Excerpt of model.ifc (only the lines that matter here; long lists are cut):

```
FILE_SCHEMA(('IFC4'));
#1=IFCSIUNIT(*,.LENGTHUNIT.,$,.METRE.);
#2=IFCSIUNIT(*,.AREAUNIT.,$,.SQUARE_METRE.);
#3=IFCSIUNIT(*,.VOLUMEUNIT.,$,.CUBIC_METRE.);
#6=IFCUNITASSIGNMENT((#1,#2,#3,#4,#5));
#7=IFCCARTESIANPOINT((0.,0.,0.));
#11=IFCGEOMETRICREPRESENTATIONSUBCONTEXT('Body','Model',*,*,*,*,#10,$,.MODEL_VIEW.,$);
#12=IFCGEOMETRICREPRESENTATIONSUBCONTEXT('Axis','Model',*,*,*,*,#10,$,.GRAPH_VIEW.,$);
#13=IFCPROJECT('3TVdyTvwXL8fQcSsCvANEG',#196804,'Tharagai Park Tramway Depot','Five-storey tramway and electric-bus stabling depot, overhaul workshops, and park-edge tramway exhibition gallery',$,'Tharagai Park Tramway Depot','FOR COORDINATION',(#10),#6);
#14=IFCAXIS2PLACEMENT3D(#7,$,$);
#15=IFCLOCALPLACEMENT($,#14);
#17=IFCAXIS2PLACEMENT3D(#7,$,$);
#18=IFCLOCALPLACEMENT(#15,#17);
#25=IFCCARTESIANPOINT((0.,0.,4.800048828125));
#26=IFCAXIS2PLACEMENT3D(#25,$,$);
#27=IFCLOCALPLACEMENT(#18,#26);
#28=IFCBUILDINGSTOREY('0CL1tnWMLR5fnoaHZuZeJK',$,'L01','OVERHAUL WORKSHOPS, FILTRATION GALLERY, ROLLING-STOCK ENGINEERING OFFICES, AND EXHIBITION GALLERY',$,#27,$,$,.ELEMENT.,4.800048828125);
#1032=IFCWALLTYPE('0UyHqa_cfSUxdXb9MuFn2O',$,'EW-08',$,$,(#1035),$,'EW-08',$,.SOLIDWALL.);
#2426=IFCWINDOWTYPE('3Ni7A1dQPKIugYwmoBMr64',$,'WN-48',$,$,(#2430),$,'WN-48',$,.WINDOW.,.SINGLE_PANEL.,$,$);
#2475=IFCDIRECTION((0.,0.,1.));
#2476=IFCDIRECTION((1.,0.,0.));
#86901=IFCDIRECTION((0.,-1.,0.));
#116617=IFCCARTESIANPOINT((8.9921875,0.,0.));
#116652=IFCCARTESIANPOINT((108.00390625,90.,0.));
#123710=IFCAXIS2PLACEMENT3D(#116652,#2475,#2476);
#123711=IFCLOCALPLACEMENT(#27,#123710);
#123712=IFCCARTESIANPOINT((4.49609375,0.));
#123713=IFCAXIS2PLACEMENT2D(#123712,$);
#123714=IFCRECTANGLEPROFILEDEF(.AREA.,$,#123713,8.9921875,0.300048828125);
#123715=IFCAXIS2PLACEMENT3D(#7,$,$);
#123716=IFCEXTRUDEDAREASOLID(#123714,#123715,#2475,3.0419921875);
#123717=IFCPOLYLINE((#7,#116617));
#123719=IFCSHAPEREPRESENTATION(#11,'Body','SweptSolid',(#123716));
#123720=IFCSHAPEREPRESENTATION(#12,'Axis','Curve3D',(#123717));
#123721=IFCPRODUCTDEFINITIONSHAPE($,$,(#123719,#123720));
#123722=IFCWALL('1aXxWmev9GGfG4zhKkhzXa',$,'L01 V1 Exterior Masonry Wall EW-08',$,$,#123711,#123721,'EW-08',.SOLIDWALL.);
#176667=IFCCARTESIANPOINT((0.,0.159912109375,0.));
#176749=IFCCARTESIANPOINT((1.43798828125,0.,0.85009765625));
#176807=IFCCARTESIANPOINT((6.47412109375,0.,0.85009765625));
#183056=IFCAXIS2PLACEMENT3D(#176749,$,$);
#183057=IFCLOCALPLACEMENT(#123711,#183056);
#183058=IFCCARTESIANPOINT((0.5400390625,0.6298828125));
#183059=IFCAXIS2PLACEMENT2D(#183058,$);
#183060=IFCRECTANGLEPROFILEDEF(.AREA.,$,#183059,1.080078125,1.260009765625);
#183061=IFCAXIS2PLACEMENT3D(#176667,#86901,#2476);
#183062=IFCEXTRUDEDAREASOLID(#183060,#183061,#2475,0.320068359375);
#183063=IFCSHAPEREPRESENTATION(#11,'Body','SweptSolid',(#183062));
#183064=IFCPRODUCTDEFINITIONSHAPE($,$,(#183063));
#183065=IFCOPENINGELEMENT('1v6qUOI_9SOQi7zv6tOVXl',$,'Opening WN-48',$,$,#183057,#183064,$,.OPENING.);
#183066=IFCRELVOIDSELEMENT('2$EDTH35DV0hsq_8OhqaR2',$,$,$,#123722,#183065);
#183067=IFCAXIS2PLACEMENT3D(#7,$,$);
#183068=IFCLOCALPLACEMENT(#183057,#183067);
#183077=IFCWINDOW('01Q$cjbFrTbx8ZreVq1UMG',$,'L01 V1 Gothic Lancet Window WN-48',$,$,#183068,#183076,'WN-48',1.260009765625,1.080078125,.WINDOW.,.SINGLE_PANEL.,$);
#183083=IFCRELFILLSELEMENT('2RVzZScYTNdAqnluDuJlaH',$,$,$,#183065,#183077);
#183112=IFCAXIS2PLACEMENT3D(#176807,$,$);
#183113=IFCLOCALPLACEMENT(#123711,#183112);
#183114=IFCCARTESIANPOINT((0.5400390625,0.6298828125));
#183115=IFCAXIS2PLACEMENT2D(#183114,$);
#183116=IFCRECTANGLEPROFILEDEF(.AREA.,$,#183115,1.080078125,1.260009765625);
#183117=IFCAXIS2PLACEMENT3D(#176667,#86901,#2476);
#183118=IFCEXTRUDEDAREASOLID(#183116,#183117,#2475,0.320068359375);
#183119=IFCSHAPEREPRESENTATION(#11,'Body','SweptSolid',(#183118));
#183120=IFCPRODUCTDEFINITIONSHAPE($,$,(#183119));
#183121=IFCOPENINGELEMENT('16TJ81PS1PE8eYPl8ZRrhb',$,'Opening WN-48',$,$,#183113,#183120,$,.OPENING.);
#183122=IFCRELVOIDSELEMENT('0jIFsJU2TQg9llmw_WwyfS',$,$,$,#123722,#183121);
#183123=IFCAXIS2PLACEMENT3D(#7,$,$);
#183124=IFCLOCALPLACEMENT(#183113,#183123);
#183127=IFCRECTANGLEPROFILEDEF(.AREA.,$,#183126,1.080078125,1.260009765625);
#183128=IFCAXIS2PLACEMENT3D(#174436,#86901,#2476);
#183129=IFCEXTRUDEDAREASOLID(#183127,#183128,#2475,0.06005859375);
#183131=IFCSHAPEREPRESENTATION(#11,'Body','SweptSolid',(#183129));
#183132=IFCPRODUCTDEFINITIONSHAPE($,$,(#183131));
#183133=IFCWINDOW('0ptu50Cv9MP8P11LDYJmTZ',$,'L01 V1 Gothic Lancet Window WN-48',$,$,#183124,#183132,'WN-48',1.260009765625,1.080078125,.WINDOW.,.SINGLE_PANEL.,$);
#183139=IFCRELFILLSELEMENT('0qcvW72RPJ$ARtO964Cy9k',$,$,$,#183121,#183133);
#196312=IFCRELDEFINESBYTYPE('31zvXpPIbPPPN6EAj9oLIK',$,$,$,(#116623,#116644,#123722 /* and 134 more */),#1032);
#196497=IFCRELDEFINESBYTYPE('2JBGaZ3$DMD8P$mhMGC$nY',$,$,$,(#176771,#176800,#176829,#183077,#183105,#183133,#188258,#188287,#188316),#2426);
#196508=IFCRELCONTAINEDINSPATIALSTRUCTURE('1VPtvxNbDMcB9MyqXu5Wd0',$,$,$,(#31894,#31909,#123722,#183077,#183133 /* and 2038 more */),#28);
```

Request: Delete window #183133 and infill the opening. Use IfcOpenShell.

```python
import ifcopenshell
import ifcopenshell.api.feature
import ifcopenshell.api.root
import ifcopenshell.geom
import ifcopenshell.util.shape

model = ifcopenshell.open("model.ifc")
settings = ifcopenshell.geom.settings()


def volume(element):
    """Net volume in cubic metres, openings subtracted."""
    shape = ifcopenshell.geom.create_shape(settings, element)
    return ifcopenshell.util.shape.get_volume(shape.geometry)


window = model.by_guid("0ptu50Cv9MP8P11LDYJmTZ")
opening = window.FillsVoids[0].RelatingOpeningElement
wall = opening.VoidsElements[0].RelatingBuildingElement
before = volume(wall)

ifcopenshell.api.root.remove_product(model, product=window)
ifcopenshell.api.feature.remove_feature(model, feature=opening)

after = volume(wall)

print(f"wall volume {before:.3f} -> {after:.3f} m3")

model.write("model_updated.ifc")
```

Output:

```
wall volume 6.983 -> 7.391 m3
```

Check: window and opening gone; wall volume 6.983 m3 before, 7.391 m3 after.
